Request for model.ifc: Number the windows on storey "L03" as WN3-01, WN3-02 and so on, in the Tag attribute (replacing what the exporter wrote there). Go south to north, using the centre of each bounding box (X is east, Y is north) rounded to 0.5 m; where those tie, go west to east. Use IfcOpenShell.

First a look at what the model holds.

```python
import ifcopenshell
import ifcopenshell.util.element
import ifcopenshell.util.placement

model = ifcopenshell.open("model.ifc")
print(model.schema)
storey = next(s for s in model.by_type("IfcBuildingStorey") if s.Name == "L03")
windows = [e for e in ifcopenshell.util.element.get_decomposition(storey) if e.is_a("IfcWindow")]
for e in sorted(windows, key=lambda e: e.id()):
    origin = ifcopenshell.util.placement.get_local_placement(e.ObjectPlacement)[:3, 3]
    print(e.id(), e.Tag, e.Name, origin.round(2) + 0.0, sep=" | ")
```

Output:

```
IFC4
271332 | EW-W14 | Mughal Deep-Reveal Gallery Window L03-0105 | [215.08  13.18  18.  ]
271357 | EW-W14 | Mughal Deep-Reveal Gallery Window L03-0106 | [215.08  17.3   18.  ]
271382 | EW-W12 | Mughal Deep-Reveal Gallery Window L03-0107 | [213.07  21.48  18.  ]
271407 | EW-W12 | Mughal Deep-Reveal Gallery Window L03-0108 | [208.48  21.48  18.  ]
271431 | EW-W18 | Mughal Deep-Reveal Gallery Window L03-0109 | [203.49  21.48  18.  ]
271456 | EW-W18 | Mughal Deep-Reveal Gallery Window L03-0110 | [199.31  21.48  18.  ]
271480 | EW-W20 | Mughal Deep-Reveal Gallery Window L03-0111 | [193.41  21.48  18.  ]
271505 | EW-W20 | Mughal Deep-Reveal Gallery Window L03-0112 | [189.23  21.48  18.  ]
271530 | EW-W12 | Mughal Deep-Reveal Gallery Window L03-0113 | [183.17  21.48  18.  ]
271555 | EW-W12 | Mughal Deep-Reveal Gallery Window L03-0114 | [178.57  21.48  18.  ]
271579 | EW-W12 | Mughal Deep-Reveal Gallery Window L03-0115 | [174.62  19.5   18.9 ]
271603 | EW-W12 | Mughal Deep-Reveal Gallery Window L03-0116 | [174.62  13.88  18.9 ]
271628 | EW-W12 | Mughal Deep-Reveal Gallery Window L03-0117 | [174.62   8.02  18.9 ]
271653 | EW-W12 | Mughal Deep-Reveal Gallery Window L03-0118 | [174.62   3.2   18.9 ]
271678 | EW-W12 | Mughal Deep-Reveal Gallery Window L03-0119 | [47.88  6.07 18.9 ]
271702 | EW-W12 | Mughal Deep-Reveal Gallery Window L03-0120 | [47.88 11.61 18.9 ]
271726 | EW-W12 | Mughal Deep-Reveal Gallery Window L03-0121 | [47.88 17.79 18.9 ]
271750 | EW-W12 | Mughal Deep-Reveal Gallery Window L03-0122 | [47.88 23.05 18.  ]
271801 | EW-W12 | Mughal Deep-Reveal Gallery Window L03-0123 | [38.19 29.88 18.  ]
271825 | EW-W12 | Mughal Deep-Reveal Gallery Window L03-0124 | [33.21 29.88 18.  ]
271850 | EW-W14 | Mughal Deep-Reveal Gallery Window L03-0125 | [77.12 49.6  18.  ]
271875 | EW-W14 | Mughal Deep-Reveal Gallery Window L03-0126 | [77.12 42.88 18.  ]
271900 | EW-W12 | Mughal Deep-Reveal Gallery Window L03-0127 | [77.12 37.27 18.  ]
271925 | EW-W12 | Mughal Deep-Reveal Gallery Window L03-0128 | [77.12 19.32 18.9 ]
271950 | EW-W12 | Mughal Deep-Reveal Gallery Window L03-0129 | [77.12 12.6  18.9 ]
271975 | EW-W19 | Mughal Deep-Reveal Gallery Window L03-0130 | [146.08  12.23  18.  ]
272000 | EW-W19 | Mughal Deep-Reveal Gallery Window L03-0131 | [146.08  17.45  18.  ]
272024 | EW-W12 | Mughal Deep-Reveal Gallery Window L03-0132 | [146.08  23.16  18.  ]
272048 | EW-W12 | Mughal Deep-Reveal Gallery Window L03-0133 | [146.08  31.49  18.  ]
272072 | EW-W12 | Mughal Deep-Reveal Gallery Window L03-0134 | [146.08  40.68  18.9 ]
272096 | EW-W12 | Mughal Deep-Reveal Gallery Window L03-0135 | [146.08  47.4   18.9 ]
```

```python
import ifcopenshell
import ifcopenshell.geom
import ifcopenshell.util.element
import ifcopenshell.util.shape

model = ifcopenshell.open("model.ifc")
settings = ifcopenshell.geom.settings()
settings.set("use-world-coords", True)


def centre(element):
    shape = ifcopenshell.geom.create_shape(settings, element)
    return ifcopenshell.util.shape.get_bbox_centroid(shape.geometry)


storey = next(s for s in model.by_type("IfcBuildingStorey") if s.Name == "L03")
windows = [e for e in ifcopenshell.util.element.get_decomposition(storey) if e.is_a("IfcWindow")]

# Insertion points can sit at a corner or the storey origin, so sort by the geometry (in metres).
centres = {e: centre(e) for e in windows}
windows.sort(key=lambda e: (round(centres[e][1] / 0.5), centres[e][0]))

for i, e in enumerate(windows, start=1):
    number = f"WN3-{i:02d}"
    e.Tag = number
    print(e.id(), number)

model.write("model_updated.ifc")
```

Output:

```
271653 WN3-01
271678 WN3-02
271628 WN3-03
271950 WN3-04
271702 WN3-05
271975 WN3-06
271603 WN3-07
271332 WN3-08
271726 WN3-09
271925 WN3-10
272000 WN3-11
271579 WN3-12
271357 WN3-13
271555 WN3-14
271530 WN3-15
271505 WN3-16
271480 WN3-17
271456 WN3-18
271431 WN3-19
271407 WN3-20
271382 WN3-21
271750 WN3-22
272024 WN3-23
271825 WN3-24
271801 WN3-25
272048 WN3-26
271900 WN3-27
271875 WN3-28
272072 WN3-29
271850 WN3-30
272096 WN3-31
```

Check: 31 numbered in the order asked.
